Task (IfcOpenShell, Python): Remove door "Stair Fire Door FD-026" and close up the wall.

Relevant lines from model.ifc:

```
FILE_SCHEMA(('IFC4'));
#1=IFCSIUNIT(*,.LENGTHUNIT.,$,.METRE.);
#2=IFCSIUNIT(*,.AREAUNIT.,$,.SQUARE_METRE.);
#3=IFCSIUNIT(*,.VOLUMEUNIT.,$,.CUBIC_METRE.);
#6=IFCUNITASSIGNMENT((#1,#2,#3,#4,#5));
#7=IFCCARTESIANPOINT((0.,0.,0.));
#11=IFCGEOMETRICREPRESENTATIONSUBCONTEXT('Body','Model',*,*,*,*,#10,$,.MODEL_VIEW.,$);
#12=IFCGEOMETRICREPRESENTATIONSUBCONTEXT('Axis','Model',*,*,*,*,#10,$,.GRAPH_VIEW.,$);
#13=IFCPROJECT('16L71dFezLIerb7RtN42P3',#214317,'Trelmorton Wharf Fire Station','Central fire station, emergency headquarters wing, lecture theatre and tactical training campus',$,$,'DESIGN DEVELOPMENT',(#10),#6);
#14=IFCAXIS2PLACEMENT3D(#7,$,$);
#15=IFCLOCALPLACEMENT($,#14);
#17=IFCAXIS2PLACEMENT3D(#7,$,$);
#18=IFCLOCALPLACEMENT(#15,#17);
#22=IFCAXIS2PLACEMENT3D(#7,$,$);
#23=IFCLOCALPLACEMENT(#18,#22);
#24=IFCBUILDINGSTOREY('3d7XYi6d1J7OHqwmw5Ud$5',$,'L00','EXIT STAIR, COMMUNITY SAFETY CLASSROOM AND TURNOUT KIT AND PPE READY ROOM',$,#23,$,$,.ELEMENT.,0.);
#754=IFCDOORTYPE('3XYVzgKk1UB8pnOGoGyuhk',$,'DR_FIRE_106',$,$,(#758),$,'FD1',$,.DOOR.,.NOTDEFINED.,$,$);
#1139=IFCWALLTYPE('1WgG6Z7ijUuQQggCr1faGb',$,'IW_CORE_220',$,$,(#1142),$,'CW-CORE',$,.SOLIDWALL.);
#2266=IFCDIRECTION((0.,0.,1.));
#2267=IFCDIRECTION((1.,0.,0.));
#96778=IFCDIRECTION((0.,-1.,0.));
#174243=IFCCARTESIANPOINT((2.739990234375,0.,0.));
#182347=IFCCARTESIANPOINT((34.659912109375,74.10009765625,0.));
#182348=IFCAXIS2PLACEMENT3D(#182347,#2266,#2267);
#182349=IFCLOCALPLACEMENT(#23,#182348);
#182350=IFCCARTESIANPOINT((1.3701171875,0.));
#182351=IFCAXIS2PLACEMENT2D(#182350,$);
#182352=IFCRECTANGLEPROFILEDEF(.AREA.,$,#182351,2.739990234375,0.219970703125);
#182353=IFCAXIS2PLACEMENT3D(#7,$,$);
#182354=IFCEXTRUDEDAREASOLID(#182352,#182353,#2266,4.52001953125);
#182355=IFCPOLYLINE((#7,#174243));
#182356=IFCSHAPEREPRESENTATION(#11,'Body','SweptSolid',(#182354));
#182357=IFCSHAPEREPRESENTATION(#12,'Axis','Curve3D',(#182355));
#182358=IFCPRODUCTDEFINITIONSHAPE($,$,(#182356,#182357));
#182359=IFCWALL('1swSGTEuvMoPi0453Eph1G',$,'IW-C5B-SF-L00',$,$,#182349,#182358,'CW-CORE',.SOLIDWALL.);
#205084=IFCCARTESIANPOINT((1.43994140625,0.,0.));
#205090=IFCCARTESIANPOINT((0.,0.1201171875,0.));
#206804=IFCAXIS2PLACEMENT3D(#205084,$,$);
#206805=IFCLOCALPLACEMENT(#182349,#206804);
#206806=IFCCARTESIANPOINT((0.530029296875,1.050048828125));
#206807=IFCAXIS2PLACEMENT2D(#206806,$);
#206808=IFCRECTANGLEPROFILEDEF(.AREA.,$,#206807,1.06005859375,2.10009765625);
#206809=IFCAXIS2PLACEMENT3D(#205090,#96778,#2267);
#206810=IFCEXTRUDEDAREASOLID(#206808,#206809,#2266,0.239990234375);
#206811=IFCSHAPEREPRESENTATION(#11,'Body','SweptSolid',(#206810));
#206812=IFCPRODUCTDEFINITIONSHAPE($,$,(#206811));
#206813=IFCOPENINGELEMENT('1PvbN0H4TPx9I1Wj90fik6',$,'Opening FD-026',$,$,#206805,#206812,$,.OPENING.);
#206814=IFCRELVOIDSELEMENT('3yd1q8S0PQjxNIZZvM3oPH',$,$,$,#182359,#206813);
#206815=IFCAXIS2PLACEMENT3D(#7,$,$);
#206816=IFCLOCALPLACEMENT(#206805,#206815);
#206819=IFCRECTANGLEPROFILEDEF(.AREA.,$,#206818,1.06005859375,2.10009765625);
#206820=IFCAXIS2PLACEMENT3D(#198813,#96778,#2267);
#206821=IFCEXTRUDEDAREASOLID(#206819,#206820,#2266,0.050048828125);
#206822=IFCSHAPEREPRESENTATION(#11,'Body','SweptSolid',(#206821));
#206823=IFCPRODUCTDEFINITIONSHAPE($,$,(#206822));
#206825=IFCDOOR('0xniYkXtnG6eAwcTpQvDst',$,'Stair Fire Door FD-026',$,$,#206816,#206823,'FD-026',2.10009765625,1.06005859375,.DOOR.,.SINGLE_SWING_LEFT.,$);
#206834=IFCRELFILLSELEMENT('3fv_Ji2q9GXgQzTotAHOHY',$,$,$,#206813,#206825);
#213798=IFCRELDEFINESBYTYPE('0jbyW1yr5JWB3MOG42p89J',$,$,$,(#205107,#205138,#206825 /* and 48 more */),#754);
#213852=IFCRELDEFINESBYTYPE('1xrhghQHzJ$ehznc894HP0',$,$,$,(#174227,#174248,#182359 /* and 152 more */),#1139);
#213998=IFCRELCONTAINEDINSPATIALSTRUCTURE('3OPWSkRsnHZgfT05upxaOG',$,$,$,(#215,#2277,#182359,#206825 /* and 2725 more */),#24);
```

```python
import ifcopenshell
import ifcopenshell.api.feature
import ifcopenshell.api.root
import ifcopenshell.geom
import ifcopenshell.util.shape

model = ifcopenshell.open("model.ifc")
settings = ifcopenshell.geom.settings()


def volume(element):
    """Net volume in cubic metres, openings subtracted."""
    shape = ifcopenshell.geom.create_shape(settings, element)
    return ifcopenshell.util.shape.get_volume(shape.geometry)


door = model.by_guid("0xniYkXtnG6eAwcTpQvDst")
opening = door.FillsVoids[0].RelatingOpeningElement
wall = opening.VoidsElements[0].RelatingBuildingElement
before = volume(wall)

ifcopenshell.api.root.remove_product(model, product=door)
ifcopenshell.api.feature.remove_feature(model, feature=opening)

after = volume(wall)

print(f"wall volume {before:.3f} -> {after:.3f} m3")

model.write("model_rev.ifc")
```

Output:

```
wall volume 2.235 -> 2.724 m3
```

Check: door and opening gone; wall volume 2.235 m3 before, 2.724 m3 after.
